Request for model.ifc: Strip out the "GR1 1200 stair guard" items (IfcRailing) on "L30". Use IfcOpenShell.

First a look at what the model holds.

```python
import ifcopenshell
import ifcopenshell.util.element

model = ifcopenshell.open("model.ifc")
print(model.schema)
storey = next(s for s in model.by_type("IfcBuildingStorey") if s.Name == "L30")
railings = [e for e in ifcopenshell.util.element.get_decomposition(storey) if e.is_a("IfcRailing")]
seen = {}
for e in railings:
    element_type = ifcopenshell.util.element.get_type(e)
    name = element_type.Name if element_type not in (None, e) else None
    seen[name] = seen.get(name, 0) + 1
for name, count in sorted(seen.items(), key=str):
    print(count, "x", name)
```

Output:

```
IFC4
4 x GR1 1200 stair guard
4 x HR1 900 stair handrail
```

```python
import ifcopenshell
import ifcopenshell.api.root
import ifcopenshell.util.element

model = ifcopenshell.open("model.ifc")

storey = next(s for s in model.by_type("IfcBuildingStorey") if s.Name == "L30")
railings = [e for e in ifcopenshell.util.element.get_decomposition(storey) if e.is_a("IfcRailing")]
targets = [e for e in railings if (t := ifcopenshell.util.element.get_type(e)) not in (None, e) and t.Name == "GR1 1200 stair guard"]

for e in targets:
    ifcopenshell.api.root.remove_product(model, product=e)
print(len(targets), "removed")

model.write("model_rev.ifc")
```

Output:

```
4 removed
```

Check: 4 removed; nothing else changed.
